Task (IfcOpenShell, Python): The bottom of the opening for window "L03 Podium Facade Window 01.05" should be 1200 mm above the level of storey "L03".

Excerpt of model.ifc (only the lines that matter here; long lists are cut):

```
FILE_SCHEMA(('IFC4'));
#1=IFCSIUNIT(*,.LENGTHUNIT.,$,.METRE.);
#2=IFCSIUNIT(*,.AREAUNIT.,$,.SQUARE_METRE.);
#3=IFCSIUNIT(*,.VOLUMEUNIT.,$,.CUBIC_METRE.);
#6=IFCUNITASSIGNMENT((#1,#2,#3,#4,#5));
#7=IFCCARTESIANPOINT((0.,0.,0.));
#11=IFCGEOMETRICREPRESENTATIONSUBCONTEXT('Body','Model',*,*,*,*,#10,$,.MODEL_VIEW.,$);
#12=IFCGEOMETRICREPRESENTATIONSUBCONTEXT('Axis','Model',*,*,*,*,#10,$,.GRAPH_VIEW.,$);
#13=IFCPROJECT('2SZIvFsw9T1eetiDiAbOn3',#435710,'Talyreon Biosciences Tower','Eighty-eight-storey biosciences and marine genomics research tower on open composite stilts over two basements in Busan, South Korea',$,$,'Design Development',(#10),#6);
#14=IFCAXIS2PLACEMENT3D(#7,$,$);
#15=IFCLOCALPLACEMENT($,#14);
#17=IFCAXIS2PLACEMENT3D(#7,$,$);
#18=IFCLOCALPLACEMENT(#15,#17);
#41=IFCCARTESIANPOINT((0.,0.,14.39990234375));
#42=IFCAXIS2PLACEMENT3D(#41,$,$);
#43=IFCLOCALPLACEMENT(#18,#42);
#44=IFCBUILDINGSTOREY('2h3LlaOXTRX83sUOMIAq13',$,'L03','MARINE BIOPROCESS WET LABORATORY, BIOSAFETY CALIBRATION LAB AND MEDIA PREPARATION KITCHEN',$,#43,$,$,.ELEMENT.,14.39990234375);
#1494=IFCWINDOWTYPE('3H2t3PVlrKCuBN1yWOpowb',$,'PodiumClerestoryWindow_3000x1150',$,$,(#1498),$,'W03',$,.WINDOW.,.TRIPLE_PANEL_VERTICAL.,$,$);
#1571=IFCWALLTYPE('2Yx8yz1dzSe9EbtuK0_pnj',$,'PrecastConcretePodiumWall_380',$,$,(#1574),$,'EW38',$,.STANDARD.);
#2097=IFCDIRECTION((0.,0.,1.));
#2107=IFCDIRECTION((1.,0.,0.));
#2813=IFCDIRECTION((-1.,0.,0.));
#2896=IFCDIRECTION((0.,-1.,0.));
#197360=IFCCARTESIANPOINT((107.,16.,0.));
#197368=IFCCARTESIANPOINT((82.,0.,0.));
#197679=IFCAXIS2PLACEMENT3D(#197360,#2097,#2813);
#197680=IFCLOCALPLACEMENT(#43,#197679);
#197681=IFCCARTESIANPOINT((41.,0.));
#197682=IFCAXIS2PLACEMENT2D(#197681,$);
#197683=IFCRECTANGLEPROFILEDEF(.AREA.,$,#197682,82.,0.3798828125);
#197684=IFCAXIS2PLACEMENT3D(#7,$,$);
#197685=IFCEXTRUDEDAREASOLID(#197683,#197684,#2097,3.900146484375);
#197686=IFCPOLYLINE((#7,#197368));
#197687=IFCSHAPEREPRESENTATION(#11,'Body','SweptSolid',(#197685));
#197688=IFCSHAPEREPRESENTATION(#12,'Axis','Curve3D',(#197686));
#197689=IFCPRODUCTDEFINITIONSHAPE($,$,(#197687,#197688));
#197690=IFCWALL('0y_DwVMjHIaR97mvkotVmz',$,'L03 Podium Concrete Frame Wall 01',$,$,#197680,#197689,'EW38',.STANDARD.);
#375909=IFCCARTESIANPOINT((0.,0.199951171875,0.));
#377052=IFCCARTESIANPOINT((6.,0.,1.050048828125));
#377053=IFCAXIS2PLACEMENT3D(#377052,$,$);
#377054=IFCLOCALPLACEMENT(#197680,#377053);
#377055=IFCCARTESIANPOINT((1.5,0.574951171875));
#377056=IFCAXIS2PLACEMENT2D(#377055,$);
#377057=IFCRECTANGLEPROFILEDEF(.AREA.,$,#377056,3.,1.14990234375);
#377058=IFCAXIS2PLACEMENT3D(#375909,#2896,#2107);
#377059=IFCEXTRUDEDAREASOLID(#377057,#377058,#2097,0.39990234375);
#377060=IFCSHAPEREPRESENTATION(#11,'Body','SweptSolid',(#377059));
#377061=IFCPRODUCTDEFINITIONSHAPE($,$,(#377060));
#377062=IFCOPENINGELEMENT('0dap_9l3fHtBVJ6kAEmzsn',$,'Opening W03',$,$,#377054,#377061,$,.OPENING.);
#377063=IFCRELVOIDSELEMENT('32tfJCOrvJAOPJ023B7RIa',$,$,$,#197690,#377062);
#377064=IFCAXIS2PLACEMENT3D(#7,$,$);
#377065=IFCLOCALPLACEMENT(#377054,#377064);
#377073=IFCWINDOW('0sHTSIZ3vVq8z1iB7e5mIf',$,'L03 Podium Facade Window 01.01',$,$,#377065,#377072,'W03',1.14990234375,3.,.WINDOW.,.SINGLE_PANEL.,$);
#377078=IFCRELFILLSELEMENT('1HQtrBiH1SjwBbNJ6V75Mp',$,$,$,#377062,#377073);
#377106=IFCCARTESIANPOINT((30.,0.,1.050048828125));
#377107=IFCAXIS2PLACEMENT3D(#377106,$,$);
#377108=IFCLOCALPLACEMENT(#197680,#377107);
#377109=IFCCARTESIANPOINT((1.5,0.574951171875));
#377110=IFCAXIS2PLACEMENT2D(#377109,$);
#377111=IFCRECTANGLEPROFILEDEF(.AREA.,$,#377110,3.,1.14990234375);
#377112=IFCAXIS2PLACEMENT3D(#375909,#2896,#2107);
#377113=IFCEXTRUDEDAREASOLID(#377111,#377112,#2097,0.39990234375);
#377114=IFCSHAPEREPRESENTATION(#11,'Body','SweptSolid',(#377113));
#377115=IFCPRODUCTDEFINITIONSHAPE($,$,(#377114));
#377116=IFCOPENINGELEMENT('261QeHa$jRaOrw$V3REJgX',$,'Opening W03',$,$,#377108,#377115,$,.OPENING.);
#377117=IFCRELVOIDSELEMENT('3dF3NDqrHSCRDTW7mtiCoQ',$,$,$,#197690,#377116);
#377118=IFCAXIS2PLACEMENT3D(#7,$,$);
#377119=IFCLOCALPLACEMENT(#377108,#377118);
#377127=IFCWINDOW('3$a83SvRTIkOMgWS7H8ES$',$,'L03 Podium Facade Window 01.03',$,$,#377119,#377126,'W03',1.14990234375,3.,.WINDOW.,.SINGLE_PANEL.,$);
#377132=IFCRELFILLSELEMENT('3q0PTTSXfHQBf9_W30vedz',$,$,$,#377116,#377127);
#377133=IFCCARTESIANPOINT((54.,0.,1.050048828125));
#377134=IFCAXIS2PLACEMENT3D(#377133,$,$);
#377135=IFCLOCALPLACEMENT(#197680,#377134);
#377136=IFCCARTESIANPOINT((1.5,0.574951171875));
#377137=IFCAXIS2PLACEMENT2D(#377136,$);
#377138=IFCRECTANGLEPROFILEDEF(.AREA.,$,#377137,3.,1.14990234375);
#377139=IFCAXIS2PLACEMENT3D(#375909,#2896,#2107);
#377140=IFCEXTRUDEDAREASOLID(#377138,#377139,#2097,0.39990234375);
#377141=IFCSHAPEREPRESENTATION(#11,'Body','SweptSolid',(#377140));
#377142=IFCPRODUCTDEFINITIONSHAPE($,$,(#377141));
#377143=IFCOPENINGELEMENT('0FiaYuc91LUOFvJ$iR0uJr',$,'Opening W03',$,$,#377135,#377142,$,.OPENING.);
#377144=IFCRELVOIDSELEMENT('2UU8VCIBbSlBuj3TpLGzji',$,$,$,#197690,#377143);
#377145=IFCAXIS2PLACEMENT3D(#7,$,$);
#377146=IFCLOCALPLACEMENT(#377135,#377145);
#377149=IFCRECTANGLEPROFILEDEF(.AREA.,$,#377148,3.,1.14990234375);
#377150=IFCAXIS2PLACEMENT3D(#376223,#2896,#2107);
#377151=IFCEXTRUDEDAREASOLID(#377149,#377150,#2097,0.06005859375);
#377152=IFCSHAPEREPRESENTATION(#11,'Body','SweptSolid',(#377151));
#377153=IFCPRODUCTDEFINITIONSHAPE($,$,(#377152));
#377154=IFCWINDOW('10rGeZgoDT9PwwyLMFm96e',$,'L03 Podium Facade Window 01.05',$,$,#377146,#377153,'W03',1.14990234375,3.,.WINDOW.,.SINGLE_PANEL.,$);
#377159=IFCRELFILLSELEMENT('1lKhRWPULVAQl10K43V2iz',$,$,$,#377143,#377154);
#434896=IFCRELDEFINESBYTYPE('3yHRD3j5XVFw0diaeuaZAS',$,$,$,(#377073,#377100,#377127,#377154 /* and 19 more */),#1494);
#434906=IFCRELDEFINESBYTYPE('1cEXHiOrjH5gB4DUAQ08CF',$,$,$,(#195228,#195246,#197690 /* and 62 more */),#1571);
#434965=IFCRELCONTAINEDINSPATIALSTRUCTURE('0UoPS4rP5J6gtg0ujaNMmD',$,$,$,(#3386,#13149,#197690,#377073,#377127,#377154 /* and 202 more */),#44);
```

```python
import numpy as np
import ifcopenshell
import ifcopenshell.api.geometry
import ifcopenshell.geom
import ifcopenshell.util.element
import ifcopenshell.util.placement
import ifcopenshell.util.shape
import ifcopenshell.util.unit

model = ifcopenshell.open("model.ifc")
unit_scale = ifcopenshell.util.unit.calculate_unit_scale(model)

window = model.by_id(377154)
opening = window.FillsVoids[0].RelatingOpeningElement
storey = ifcopenshell.util.element.get_container(window, ifc_class="IfcBuildingStorey")
level = ifcopenshell.util.placement.get_local_placement(storey.ObjectPlacement)[2, 3]

# The opening's origin need not be at the sill, so measure its lowest point.
shape = ifcopenshell.geom.create_shape(ifcopenshell.geom.settings(), opening)
bottom = ifcopenshell.util.shape.get_shape_bottom_elevation(shape, shape.geometry) / unit_scale
dz = level + 1.2 - bottom

shift = np.array([0.0, 0.0, dz])
# The window is placed relative to its opening, so it follows when the opening moves.
matrix = ifcopenshell.util.placement.get_local_placement(opening.ObjectPlacement)
matrix[:3, 3] += shift
ifcopenshell.api.geometry.edit_object_placement(
    model, product=opening, matrix=matrix, is_si=False, should_transform_children=True
)

print(f"moved by {dz * unit_scale:+.3f} m")

model.write("model_v2.ifc")
```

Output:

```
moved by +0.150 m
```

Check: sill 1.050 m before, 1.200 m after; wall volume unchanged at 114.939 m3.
